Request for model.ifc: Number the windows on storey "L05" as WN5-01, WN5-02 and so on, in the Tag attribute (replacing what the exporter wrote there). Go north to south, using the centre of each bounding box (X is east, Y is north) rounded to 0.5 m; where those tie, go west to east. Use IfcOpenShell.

First a look at what the model holds.

```python
import ifcopenshell
import ifcopenshell.util.element
import ifcopenshell.util.placement

model = ifcopenshell.open("model.ifc")
print(model.schema)
storey = next(s for s in model.by_type("IfcBuildingStorey") if s.Name == "L05")
windows = [e for e in ifcopenshell.util.element.get_decomposition(storey) if e.is_a("IfcWindow")]
for e in sorted(windows, key=lambda e: e.id()):
    origin = ifcopenshell.util.placement.get_local_placement(e.ObjectPlacement)[:3, 3]
    print(e.id(), e.Tag, e.Name, origin.round(2) + 0.0, sep=" | ")
```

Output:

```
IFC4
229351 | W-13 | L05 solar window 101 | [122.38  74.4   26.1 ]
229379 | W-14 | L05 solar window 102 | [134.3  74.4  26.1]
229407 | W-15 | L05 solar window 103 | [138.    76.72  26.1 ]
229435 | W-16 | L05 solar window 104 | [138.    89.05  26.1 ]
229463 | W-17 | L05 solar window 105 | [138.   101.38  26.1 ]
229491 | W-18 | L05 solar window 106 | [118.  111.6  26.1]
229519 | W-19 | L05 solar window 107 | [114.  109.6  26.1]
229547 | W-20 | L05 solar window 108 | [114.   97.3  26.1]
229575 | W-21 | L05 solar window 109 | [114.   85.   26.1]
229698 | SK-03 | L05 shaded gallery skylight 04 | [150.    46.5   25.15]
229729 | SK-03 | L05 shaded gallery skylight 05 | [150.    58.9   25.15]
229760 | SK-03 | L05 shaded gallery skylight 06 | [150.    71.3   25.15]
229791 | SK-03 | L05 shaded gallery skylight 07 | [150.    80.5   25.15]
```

```python
import ifcopenshell
import ifcopenshell.geom
import ifcopenshell.util.element
import ifcopenshell.util.shape

model = ifcopenshell.open("model.ifc")
settings = ifcopenshell.geom.settings()
settings.set("use-world-coords", True)


def centre(element):
    shape = ifcopenshell.geom.create_shape(settings, element)
    return ifcopenshell.util.shape.get_bbox_centroid(shape.geometry)


storey = next(s for s in model.by_type("IfcBuildingStorey") if s.Name == "L05")
windows = [e for e in ifcopenshell.util.element.get_decomposition(storey) if e.is_a("IfcWindow")]

# Insertion points can sit at a corner or the storey origin, so sort by the geometry (in metres).
centres = {e: centre(e) for e in windows}
windows.sort(key=lambda e: (-round(centres[e][1] / 0.5), centres[e][0]))

for i, e in enumerate(windows, start=1):
    number = f"WN5-{i:02d}"
    e.Tag = number
    print(e.id(), number)

model.write("model_v2.ifc")
```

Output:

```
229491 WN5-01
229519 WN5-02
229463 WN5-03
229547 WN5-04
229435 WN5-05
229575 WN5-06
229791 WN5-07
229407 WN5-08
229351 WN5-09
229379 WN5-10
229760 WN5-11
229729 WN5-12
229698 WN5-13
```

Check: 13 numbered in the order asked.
